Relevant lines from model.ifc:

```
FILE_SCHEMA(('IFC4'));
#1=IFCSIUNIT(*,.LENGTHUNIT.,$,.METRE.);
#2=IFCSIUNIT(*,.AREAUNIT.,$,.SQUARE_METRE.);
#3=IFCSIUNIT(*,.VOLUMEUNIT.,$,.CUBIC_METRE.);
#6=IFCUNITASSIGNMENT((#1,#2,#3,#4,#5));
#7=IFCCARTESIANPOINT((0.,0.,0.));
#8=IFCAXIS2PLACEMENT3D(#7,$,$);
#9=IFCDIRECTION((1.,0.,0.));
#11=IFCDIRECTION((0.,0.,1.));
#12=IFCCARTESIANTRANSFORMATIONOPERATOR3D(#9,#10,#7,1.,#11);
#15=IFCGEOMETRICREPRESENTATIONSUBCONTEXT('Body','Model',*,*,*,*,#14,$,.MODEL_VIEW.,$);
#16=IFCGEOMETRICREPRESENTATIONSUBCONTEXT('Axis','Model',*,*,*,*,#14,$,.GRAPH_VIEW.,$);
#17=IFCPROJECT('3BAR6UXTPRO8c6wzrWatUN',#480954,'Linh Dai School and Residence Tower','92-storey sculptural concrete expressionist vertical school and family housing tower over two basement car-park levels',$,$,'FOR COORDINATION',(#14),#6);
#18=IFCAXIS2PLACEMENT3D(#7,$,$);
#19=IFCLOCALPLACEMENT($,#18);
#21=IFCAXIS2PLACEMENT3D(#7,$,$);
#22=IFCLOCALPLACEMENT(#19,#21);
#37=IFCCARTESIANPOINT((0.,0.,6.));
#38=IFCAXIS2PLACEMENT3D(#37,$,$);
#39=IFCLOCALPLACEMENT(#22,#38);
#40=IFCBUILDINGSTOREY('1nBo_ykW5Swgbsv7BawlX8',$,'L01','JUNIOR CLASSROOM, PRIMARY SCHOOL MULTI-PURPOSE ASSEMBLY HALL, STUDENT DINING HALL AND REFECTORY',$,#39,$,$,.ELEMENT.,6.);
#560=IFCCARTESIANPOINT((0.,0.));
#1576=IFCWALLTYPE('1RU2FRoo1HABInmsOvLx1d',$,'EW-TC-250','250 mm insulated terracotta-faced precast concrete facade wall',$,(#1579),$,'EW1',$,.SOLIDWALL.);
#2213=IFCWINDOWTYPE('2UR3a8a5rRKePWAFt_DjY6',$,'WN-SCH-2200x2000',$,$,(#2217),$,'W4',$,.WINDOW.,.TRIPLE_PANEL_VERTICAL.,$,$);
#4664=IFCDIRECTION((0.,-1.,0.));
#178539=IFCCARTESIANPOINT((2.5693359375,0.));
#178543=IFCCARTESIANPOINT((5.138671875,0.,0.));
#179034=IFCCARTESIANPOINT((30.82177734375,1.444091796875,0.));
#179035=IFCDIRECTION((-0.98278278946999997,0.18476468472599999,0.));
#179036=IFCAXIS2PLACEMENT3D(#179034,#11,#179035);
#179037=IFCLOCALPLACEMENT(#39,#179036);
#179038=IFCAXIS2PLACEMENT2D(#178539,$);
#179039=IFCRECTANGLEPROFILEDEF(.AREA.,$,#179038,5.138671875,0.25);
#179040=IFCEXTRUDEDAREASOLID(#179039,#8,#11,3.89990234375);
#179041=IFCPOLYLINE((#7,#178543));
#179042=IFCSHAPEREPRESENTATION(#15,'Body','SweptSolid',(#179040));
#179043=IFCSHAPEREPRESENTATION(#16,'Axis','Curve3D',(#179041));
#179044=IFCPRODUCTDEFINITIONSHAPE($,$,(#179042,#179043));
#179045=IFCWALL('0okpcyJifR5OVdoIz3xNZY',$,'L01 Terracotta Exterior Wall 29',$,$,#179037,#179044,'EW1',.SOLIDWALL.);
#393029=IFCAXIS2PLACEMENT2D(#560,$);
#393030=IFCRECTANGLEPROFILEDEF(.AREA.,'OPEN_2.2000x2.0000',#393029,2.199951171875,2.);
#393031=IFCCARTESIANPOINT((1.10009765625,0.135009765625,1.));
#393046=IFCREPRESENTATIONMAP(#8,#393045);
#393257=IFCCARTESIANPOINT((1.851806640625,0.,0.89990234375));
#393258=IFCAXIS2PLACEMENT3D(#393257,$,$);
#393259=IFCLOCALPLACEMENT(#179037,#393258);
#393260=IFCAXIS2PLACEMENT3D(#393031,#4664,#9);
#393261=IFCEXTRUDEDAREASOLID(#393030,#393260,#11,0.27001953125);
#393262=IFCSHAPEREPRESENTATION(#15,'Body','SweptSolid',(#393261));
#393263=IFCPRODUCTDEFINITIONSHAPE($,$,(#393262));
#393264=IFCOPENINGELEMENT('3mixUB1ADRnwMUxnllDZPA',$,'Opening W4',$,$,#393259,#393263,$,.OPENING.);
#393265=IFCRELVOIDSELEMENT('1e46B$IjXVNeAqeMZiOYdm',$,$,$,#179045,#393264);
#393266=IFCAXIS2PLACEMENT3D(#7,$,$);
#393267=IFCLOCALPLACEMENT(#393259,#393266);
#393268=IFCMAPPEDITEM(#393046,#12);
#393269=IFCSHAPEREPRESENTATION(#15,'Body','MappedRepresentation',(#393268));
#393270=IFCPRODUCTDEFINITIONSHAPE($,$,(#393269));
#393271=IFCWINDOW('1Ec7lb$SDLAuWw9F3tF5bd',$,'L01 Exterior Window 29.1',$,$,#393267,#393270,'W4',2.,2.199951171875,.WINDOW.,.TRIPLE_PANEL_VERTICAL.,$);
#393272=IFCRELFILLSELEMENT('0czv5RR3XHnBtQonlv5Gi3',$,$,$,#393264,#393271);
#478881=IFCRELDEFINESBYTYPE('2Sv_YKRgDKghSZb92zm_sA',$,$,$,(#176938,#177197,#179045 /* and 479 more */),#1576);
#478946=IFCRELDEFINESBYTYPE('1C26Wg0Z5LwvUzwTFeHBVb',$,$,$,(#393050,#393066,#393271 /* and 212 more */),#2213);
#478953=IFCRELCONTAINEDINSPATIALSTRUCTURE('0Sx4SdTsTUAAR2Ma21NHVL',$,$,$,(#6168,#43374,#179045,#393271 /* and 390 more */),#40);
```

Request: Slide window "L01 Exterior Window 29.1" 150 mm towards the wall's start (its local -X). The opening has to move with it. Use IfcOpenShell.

```python
import ifcopenshell
import ifcopenshell.api.geometry
import ifcopenshell.util.placement
import ifcopenshell.util.unit

model = ifcopenshell.open("model.ifc")
unit_scale = ifcopenshell.util.unit.calculate_unit_scale(model)

window = model.by_guid("1Ec7lb$SDLAuWw9F3tF5bd")
opening = window.FillsVoids[0].RelatingOpeningElement
wall = opening.VoidsElements[0].RelatingBuildingElement

wall_matrix = ifcopenshell.util.placement.get_local_placement(wall.ObjectPlacement)
shift = wall_matrix[:3, 0] * -0.15 / unit_scale
before = ifcopenshell.util.placement.get_local_placement(window.ObjectPlacement)[:3, 3].copy()

# The window is placed relative to its opening, so it follows when the opening moves.
matrix = ifcopenshell.util.placement.get_local_placement(opening.ObjectPlacement)
matrix[:3, 3] += shift
ifcopenshell.api.geometry.edit_object_placement(
    model, product=opening, matrix=matrix, is_si=False, should_transform_children=True
)

after = ifcopenshell.util.placement.get_local_placement(window.ObjectPlacement)[:3, 3]
print("window moved by", (after - before).round(3) + 0.0)

model.write("model_v2.ifc")
```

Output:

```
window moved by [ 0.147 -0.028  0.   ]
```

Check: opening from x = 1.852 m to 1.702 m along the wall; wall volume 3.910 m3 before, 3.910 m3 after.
